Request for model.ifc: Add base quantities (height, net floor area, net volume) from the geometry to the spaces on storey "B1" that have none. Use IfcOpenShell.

First a look at what the model holds.

```python
import ifcopenshell
import ifcopenshell.util.element
import ifcopenshell.util.unit

model = ifcopenshell.open("model.ifc")
print(model.schema)
for unit_type in ("LENGTHUNIT", "AREAUNIT", "VOLUMEUNIT"):
    print(unit_type, ifcopenshell.util.unit.calculate_unit_scale(model, unit_type))
storey = next(s for s in model.by_type("IfcBuildingStorey") if s.Name == "B1")
spaces = [e for e in ifcopenshell.util.element.get_decomposition(storey) if e.is_a("IfcSpace")]
for e in sorted(spaces, key=lambda e: e.id()):
    print(e.id(), e.is_a(), e.Name, list(ifcopenshell.util.element.get_psets(e, qtos_only=True)), sep=" | ")
```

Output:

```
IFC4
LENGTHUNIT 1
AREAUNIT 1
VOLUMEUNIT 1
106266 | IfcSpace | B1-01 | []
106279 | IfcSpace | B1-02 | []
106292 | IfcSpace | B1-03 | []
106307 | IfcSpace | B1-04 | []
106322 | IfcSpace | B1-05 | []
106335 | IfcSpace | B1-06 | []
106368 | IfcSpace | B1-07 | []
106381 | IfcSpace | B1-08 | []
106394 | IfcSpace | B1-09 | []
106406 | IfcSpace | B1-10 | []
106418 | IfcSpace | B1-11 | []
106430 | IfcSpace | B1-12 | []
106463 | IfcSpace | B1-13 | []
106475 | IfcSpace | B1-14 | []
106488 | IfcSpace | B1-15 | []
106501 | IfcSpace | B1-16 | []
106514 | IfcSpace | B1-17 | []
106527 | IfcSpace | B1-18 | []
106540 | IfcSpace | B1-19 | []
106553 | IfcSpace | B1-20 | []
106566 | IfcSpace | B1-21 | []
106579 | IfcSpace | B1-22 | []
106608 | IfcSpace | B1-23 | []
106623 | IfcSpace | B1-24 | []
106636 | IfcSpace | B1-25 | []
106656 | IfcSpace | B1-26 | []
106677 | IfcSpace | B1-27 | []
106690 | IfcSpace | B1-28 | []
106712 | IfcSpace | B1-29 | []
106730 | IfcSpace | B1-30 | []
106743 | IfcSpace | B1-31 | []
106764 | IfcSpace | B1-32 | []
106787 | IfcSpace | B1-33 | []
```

```python
import ifcopenshell
import ifcopenshell.api.pset
import ifcopenshell.geom
import ifcopenshell.util.element
import ifcopenshell.util.shape
import ifcopenshell.util.unit

model = ifcopenshell.open("model.ifc")
unit_scale = ifcopenshell.util.unit.calculate_unit_scale(model)
area_scale = ifcopenshell.util.unit.calculate_unit_scale(model, "AREAUNIT")
volume_scale = ifcopenshell.util.unit.calculate_unit_scale(model, "VOLUMEUNIT")
settings = ifcopenshell.geom.settings()

storey = next(s for s in model.by_type("IfcBuildingStorey") if s.Name == "B1")
spaces = [e for e in ifcopenshell.util.element.get_decomposition(storey) if e.is_a("IfcSpace")]

for e in sorted(spaces, key=lambda e: e.id()):
    if ifcopenshell.util.element.get_psets(e, qtos_only=True, should_inherit=False):
        continue
    # Geometry comes back in metres, in the element's own axes.
    shape = ifcopenshell.geom.create_shape(settings, e)
    values = {
        "Height": ifcopenshell.util.shape.get_z(shape.geometry) / unit_scale,
        "NetFloorArea": ifcopenshell.util.shape.get_footprint_area(shape.geometry) / area_scale,
        "NetVolume": ifcopenshell.util.shape.get_volume(shape.geometry) / volume_scale,
    }
    qto = ifcopenshell.api.pset.add_qto(model, product=e, name="Qto_SpaceBaseQuantities")
    ifcopenshell.api.pset.edit_qto(model, qto=qto, properties=values)
    print(e.id(), {k: round(v, 3) for k, v in values.items()})

model.write("model_updated.ifc")
```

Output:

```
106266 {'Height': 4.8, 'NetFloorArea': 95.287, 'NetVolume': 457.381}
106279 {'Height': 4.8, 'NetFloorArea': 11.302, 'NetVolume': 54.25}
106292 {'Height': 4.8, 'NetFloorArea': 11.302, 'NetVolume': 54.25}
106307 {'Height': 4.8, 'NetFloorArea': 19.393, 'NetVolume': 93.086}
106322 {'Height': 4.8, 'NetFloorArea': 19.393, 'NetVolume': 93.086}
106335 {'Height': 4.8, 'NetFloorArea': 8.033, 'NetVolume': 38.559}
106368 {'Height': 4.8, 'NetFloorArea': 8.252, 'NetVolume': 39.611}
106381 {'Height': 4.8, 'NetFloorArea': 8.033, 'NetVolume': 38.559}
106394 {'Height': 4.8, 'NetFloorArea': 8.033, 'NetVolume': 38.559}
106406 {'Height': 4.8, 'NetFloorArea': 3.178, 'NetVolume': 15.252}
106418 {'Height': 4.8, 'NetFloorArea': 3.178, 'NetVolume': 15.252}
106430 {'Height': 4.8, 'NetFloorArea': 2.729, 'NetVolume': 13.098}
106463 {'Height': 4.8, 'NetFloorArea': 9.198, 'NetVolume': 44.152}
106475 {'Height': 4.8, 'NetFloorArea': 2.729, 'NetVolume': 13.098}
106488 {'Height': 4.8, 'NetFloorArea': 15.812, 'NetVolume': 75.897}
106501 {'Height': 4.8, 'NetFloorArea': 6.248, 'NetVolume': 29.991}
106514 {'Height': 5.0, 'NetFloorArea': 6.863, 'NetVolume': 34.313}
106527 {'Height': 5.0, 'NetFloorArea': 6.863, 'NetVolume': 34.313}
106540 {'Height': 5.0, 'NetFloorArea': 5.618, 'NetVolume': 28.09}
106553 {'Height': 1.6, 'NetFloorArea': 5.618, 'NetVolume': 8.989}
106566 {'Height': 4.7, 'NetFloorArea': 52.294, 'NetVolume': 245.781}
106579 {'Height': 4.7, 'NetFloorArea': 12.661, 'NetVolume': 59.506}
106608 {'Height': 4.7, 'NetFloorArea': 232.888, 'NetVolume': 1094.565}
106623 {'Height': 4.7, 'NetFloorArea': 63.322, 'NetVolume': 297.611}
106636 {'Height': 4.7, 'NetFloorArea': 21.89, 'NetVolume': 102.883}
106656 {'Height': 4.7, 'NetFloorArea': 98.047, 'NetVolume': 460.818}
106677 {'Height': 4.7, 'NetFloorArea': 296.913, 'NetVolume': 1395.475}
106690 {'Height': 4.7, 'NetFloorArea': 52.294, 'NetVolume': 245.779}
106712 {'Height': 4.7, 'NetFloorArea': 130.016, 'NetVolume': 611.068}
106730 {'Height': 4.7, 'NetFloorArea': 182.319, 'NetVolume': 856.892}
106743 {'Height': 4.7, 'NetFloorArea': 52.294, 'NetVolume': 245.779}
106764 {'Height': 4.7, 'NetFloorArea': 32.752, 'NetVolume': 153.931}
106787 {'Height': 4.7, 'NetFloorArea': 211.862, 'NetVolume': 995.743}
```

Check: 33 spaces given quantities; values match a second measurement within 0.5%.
